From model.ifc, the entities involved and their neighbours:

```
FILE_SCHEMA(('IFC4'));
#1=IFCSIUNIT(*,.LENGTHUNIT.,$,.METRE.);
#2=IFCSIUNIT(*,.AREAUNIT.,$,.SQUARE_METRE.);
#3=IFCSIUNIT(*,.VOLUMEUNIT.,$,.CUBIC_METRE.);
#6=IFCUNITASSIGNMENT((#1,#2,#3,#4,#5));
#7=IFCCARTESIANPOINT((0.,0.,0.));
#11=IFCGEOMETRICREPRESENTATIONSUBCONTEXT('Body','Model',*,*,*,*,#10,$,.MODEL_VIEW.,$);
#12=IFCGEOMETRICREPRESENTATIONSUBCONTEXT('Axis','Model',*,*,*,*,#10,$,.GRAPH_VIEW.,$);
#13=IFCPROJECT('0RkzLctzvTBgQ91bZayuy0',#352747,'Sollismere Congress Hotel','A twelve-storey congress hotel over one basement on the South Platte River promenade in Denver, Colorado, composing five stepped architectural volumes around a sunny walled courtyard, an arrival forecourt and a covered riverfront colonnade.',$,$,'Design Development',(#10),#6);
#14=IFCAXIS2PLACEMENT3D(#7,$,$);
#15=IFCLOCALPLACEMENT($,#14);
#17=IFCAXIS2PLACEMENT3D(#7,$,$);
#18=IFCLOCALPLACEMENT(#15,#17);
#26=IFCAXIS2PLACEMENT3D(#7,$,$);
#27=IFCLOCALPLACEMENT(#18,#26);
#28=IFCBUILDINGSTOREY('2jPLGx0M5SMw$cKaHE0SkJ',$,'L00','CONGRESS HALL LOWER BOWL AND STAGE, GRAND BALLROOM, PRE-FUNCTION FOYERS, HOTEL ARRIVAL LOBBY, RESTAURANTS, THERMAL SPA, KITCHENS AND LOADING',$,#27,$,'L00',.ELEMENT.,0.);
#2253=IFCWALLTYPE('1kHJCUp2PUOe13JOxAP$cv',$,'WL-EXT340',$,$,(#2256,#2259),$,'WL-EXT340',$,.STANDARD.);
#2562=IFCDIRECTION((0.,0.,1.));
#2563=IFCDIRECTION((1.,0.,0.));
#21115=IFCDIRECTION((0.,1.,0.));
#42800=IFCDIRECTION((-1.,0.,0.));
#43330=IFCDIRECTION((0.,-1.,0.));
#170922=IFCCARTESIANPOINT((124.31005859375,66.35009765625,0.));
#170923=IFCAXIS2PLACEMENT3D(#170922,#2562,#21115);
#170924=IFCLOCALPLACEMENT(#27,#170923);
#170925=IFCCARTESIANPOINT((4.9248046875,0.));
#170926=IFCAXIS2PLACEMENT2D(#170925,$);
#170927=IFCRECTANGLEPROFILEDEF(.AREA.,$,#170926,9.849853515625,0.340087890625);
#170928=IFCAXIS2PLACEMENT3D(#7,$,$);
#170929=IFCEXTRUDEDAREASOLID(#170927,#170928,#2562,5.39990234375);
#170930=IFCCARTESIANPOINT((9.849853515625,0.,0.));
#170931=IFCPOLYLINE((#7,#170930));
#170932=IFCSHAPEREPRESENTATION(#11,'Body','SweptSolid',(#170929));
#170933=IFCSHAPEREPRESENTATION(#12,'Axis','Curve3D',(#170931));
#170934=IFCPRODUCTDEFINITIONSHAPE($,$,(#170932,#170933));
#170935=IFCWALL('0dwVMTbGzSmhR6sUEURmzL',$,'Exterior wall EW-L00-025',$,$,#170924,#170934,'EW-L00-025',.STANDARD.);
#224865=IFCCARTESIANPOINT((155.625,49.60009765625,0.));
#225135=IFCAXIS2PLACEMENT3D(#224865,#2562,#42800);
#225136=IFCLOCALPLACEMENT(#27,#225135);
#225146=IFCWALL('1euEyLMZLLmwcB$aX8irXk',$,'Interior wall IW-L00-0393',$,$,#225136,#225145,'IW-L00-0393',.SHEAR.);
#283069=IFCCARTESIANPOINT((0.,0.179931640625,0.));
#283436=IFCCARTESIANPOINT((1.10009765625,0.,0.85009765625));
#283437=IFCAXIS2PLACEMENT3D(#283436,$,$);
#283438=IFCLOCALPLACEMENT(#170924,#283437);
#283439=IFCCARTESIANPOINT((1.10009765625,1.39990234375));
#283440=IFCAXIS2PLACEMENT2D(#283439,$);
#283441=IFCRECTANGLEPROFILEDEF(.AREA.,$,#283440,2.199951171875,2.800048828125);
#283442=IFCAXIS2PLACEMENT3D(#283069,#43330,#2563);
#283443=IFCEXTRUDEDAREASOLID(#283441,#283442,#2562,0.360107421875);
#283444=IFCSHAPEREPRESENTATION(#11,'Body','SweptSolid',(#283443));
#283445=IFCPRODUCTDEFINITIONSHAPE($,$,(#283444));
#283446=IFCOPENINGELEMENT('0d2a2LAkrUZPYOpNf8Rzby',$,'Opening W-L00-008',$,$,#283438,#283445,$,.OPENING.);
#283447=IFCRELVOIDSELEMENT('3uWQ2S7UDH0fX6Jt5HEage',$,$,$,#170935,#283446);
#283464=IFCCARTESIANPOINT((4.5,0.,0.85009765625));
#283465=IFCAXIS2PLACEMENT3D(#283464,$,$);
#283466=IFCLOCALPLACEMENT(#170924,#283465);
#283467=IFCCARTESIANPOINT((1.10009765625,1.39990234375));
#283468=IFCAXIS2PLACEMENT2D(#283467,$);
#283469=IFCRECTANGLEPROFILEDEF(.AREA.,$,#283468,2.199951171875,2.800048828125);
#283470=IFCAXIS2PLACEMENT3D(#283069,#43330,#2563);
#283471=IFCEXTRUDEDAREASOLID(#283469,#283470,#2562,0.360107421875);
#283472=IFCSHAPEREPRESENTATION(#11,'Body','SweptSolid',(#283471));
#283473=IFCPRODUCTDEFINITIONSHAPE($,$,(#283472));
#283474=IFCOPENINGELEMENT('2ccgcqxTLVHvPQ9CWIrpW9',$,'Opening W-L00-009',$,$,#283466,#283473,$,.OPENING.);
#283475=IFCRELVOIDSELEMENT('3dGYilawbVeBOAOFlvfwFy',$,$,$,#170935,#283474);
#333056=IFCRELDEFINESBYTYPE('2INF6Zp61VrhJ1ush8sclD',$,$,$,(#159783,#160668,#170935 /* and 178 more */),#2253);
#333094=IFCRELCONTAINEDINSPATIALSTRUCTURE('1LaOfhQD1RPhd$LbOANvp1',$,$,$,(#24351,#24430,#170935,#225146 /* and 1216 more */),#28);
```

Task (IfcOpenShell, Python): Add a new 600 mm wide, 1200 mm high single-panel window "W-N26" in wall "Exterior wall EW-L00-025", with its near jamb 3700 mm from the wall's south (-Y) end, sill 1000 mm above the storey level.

```python
import numpy as np
import ifcopenshell
import ifcopenshell.api.feature
import ifcopenshell.api.geometry
import ifcopenshell.api.root
import ifcopenshell.api.spatial
import ifcopenshell.geom
import ifcopenshell.util.element
import ifcopenshell.util.placement
import ifcopenshell.util.representation
import ifcopenshell.util.shape
import ifcopenshell.util.unit

model = ifcopenshell.open("model.ifc")
unit_scale = ifcopenshell.util.unit.calculate_unit_scale(model)
settings = ifcopenshell.geom.settings()


def volume(element):
    """Net volume in cubic metres, openings subtracted."""
    shape = ifcopenshell.geom.create_shape(settings, element)
    return ifcopenshell.util.shape.get_volume(shape.geometry)


wall = model.by_id(170935)
storey = ifcopenshell.util.element.get_container(wall, ifc_class="IfcBuildingStorey")
context = ifcopenshell.util.representation.get_context(model, "Model", "Body", "MODEL_VIEW")
before = volume(wall)

width, height, from_end, sill = 0.6, 1.2, 3.7, 1  # metres

# The wall runs along its own X axis, and the end named is its -X end.
wall_shape = ifcopenshell.geom.create_shape(settings, wall)
x, y, z = ifcopenshell.util.shape.get_vertices(wall_shape.geometry).T
start = x.min() + from_end
face, thickness = float(y.min()), float(y.max() - y.min())
wall_matrix = ifcopenshell.util.placement.get_local_placement(wall.ObjectPlacement)
level = ifcopenshell.util.placement.get_local_placement(storey.ObjectPlacement)[2, 3]


def in_wall(x, y):
    """Placement at x, y metres in the wall's axes, at sill height."""
    matrix = wall_matrix.copy()
    matrix[:, 3] = wall_matrix @ np.array([x / unit_scale, y / unit_scale, 0.0, 1.0])
    matrix[2, 3] = level + sill / unit_scale
    return matrix


# Opening: a box that overshoots both wall faces by 50 mm.
opening = ifcopenshell.api.root.create_entity(model, ifc_class="IfcOpeningElement", predefined_type="OPENING")
box = ifcopenshell.api.geometry.add_wall_representation(
    model, context=context, length=width, height=height, thickness=thickness + 0.1
)
ifcopenshell.api.geometry.assign_representation(model, product=opening, representation=box)
ifcopenshell.api.geometry.edit_object_placement(model, product=opening, matrix=in_wall(start, face - 0.05), is_si=False)
ifcopenshell.api.feature.add_feature(model, feature=opening, element=wall)

window = ifcopenshell.api.root.create_entity(model, ifc_class="IfcWindow", name="W-N26", predefined_type="WINDOW")
window.OverallWidth, window.OverallHeight = width / unit_scale, height / unit_scale
window.PartitioningType = "SINGLE_PANEL"
body = ifcopenshell.api.geometry.add_window_representation(
    model,
    context=context,
    overall_width=window.OverallWidth,
    overall_height=window.OverallHeight,
    partition_type="SINGLE_PANEL",
)
ifcopenshell.api.geometry.assign_representation(model, product=window, representation=body)
ifcopenshell.api.spatial.assign_container(model, products=[window], relating_structure=storey)
ifcopenshell.api.feature.add_filling(model, opening=opening, element=window)

# Centre the window in the wall's thickness.
ifcopenshell.api.geometry.edit_object_placement(model, product=window, matrix=in_wall(start, face), is_si=False)
window_shape = ifcopenshell.geom.create_shape(settings, window)
depth = ifcopenshell.util.shape.get_vertices(window_shape.geometry)[:, 1]
offset = face + thickness / 2 - (depth.min() + depth.max()) / 2
ifcopenshell.api.geometry.edit_object_placement(model, product=window, matrix=in_wall(start, offset), is_si=False)

after = volume(wall)

print(f"wall volume {before:.3f} -> {after:.3f} m3")

model.write("model_updated.ifc")
```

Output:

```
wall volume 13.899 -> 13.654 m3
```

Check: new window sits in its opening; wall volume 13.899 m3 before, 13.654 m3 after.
